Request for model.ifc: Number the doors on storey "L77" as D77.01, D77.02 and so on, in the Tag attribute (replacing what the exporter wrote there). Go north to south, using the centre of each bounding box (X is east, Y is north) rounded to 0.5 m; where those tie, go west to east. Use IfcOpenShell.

First a look at what the model holds.

```python
import ifcopenshell
import ifcopenshell.util.element
import ifcopenshell.util.placement

model = ifcopenshell.open("model.ifc")
print(model.schema)
storey = next(s for s in model.by_type("IfcBuildingStorey") if s.Name == "L77")
doors = [e for e in ifcopenshell.util.element.get_decomposition(storey) if e.is_a("IfcDoor")]
for e in sorted(doors, key=lambda e: e.id()):
    origin = ifcopenshell.util.placement.get_local_placement(e.ObjectPlacement)[:3, 3]
    print(e.id(), e.Tag, e.Name, origin.round(2) + 0.0, sep=" | ")
```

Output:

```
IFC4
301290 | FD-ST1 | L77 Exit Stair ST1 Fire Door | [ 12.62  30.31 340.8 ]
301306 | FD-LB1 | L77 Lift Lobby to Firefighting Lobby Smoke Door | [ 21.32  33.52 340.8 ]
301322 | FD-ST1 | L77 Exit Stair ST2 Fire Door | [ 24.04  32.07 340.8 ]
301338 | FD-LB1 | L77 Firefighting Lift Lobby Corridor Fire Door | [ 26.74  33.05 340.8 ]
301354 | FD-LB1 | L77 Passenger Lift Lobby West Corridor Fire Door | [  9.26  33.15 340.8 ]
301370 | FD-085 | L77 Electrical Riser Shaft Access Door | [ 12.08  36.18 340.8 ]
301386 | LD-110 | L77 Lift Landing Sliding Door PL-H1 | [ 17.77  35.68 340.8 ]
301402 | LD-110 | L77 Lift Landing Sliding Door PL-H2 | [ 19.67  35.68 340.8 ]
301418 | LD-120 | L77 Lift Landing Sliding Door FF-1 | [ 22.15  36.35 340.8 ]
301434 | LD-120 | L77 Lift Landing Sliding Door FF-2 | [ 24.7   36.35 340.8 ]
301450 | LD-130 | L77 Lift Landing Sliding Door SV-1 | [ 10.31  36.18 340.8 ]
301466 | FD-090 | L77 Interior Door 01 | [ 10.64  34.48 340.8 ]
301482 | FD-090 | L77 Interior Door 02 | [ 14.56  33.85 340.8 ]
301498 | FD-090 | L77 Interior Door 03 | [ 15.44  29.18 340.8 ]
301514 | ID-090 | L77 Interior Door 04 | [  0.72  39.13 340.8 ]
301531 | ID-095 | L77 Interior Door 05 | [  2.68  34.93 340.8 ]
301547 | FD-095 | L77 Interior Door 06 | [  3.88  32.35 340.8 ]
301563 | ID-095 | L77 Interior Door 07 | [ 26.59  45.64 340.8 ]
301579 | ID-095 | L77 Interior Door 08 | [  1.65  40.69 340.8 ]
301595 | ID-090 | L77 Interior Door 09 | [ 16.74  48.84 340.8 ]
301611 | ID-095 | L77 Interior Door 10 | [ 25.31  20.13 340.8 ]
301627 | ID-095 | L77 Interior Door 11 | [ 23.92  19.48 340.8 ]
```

```python
import ifcopenshell
import ifcopenshell.geom
import ifcopenshell.util.element
import ifcopenshell.util.shape

model = ifcopenshell.open("model.ifc")
settings = ifcopenshell.geom.settings()
settings.set("use-world-coords", True)


def centre(element):
    shape = ifcopenshell.geom.create_shape(settings, element)
    return ifcopenshell.util.shape.get_bbox_centroid(shape.geometry)


storey = next(s for s in model.by_type("IfcBuildingStorey") if s.Name == "L77")
doors = [e for e in ifcopenshell.util.element.get_decomposition(storey) if e.is_a("IfcDoor")]

# Insertion points can sit at a corner or the storey origin, so sort by the geometry (in metres).
centres = {e: centre(e) for e in doors}
doors.sort(key=lambda e: (-round(centres[e][1] / 0.5), centres[e][0]))

for i, e in enumerate(doors, start=1):
    number = f"D77.{i:02d}"
    e.Tag = number
    print(e.id(), number)

model.write("model_edited.ifc")
```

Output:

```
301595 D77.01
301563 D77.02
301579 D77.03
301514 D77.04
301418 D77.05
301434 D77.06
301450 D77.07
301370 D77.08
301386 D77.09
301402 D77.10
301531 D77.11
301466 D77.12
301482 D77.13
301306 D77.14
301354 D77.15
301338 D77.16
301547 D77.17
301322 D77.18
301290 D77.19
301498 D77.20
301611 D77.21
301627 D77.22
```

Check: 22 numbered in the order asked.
